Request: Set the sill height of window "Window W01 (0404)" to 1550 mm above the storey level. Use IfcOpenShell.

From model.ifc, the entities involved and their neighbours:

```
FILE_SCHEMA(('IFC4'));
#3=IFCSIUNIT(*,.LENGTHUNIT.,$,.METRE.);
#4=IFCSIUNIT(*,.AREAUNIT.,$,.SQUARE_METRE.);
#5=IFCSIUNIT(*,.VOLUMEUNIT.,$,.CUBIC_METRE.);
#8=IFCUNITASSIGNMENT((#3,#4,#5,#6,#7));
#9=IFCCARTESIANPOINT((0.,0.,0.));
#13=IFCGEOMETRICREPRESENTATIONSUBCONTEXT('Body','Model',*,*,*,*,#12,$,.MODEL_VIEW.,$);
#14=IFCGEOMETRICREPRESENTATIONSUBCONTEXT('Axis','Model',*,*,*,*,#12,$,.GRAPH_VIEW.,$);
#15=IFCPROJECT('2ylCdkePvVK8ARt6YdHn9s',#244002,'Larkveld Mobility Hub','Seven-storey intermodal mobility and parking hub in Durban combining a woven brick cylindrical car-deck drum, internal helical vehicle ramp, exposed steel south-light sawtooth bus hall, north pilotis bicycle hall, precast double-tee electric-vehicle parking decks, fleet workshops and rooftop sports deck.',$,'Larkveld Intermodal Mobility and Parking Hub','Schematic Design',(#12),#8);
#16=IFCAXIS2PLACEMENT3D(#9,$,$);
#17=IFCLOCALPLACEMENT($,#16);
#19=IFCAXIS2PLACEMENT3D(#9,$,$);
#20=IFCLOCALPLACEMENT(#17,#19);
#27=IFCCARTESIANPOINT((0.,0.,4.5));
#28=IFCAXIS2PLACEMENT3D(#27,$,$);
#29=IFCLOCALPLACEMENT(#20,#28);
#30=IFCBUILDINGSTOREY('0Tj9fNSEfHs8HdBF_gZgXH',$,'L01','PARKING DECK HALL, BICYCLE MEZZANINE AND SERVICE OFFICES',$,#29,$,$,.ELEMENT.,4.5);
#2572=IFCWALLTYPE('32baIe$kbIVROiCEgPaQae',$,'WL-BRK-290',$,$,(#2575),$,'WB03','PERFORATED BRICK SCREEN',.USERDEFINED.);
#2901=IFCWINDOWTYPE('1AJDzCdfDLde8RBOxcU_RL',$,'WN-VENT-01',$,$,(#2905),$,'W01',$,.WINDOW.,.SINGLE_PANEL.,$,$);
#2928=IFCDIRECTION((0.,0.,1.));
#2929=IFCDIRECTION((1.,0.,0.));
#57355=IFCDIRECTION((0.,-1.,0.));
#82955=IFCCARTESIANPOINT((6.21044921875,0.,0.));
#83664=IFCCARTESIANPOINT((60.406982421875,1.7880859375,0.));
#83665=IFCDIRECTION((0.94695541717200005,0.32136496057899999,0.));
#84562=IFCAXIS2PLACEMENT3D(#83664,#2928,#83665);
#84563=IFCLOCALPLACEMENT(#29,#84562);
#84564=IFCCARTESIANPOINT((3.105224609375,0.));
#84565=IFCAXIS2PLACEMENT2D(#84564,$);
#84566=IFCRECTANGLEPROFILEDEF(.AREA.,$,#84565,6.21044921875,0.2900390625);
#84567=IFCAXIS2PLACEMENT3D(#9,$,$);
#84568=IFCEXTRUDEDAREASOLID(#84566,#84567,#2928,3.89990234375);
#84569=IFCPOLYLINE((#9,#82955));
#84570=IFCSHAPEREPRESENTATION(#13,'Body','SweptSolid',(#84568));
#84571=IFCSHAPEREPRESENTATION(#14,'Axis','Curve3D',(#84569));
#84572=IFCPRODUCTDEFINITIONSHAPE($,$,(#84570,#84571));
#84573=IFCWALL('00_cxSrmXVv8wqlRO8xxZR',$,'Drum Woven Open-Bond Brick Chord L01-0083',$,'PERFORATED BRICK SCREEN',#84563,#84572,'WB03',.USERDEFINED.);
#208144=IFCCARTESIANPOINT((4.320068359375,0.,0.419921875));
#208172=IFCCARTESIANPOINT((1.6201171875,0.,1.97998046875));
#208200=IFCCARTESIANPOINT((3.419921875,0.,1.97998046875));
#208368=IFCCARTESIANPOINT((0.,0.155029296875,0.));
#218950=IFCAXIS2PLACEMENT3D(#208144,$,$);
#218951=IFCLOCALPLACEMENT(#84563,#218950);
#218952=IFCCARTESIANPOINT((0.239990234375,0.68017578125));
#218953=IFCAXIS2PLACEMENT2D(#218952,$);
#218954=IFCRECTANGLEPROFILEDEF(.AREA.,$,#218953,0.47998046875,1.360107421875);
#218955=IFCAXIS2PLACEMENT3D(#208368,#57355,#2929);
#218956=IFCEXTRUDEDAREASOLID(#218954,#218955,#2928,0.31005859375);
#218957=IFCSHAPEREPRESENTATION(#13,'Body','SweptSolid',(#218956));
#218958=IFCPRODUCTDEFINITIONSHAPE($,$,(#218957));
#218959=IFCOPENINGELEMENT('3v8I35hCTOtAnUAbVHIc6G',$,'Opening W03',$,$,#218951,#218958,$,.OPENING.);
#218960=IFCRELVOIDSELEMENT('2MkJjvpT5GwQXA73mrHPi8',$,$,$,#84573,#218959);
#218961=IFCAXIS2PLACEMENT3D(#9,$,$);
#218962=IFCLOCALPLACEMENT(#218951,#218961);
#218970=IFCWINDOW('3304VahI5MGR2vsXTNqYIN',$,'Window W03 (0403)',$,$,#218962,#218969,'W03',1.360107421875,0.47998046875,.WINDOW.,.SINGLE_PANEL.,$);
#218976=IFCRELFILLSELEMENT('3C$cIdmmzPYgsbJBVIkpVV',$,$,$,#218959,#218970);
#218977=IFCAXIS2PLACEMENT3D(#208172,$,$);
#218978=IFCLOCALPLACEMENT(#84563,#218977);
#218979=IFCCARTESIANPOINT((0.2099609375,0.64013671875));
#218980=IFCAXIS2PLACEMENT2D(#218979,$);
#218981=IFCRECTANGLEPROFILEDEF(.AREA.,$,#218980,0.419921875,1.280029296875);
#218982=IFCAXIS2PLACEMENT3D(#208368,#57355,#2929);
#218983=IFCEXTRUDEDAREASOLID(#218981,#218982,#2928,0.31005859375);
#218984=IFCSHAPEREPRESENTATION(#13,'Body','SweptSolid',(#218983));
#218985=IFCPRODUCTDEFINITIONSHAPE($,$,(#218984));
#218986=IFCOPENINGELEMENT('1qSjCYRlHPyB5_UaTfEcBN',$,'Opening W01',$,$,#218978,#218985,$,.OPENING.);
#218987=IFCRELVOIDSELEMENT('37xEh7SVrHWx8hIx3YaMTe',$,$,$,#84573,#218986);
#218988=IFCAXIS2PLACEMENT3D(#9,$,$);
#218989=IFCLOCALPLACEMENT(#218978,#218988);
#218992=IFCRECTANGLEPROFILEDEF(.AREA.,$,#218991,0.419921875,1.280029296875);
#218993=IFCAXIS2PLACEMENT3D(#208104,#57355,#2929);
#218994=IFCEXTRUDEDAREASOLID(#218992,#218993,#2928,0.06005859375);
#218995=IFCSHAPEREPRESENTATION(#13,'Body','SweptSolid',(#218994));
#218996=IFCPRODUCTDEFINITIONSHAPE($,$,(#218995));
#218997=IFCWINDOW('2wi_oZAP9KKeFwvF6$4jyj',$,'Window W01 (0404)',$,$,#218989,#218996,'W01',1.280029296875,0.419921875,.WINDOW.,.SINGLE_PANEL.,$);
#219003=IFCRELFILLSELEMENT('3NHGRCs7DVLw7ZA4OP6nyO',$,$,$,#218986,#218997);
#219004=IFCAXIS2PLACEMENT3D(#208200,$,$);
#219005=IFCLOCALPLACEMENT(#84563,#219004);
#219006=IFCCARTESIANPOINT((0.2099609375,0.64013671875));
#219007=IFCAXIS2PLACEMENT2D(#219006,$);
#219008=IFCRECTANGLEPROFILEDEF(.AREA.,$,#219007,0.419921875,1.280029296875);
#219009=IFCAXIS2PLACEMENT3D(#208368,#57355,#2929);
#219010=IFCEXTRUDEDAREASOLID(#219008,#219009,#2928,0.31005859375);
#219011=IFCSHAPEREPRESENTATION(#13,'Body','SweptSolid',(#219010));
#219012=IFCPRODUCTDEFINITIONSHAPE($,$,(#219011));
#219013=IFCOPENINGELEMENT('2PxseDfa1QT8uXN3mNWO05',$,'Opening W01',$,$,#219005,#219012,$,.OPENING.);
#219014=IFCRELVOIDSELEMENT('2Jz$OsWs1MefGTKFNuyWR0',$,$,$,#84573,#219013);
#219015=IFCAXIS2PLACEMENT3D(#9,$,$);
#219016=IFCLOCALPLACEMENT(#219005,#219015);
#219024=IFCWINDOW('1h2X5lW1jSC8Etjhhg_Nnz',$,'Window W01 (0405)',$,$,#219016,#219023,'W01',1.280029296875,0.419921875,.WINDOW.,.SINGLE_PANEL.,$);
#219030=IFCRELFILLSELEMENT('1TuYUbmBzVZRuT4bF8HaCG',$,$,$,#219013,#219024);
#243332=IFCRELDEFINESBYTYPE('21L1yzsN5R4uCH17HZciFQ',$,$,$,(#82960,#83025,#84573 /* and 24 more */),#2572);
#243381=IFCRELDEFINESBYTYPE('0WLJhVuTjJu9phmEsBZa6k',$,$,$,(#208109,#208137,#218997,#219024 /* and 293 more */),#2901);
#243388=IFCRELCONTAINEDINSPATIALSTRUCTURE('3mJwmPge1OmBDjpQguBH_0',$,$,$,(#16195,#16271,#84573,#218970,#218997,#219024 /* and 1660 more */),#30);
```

```python
import numpy as np
import ifcopenshell
import ifcopenshell.api.geometry
import ifcopenshell.geom
import ifcopenshell.util.element
import ifcopenshell.util.placement
import ifcopenshell.util.shape
import ifcopenshell.util.unit

model = ifcopenshell.open("model.ifc")
unit_scale = ifcopenshell.util.unit.calculate_unit_scale(model)

window = model.by_guid("2wi_oZAP9KKeFwvF6$4jyj")
opening = window.FillsVoids[0].RelatingOpeningElement
storey = ifcopenshell.util.element.get_container(window, ifc_class="IfcBuildingStorey")
level = ifcopenshell.util.placement.get_local_placement(storey.ObjectPlacement)[2, 3]

# The opening's origin need not be at the sill, so measure its lowest point.
shape = ifcopenshell.geom.create_shape(ifcopenshell.geom.settings(), opening)
bottom = ifcopenshell.util.shape.get_shape_bottom_elevation(shape, shape.geometry) / unit_scale
dz = level + 1.55 / unit_scale - bottom

shift = np.array([0.0, 0.0, dz])
# The window is placed relative to its opening, so it follows when the opening moves.
matrix = ifcopenshell.util.placement.get_local_placement(opening.ObjectPlacement)
matrix[:3, 3] += shift
ifcopenshell.api.geometry.edit_object_placement(
    model, product=opening, matrix=matrix, is_si=False, should_transform_children=True
)

print(f"moved by {dz * unit_scale:+.3f} m")

model.write("model-out.ifc")
```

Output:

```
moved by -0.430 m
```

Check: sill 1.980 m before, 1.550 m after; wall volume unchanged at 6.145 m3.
